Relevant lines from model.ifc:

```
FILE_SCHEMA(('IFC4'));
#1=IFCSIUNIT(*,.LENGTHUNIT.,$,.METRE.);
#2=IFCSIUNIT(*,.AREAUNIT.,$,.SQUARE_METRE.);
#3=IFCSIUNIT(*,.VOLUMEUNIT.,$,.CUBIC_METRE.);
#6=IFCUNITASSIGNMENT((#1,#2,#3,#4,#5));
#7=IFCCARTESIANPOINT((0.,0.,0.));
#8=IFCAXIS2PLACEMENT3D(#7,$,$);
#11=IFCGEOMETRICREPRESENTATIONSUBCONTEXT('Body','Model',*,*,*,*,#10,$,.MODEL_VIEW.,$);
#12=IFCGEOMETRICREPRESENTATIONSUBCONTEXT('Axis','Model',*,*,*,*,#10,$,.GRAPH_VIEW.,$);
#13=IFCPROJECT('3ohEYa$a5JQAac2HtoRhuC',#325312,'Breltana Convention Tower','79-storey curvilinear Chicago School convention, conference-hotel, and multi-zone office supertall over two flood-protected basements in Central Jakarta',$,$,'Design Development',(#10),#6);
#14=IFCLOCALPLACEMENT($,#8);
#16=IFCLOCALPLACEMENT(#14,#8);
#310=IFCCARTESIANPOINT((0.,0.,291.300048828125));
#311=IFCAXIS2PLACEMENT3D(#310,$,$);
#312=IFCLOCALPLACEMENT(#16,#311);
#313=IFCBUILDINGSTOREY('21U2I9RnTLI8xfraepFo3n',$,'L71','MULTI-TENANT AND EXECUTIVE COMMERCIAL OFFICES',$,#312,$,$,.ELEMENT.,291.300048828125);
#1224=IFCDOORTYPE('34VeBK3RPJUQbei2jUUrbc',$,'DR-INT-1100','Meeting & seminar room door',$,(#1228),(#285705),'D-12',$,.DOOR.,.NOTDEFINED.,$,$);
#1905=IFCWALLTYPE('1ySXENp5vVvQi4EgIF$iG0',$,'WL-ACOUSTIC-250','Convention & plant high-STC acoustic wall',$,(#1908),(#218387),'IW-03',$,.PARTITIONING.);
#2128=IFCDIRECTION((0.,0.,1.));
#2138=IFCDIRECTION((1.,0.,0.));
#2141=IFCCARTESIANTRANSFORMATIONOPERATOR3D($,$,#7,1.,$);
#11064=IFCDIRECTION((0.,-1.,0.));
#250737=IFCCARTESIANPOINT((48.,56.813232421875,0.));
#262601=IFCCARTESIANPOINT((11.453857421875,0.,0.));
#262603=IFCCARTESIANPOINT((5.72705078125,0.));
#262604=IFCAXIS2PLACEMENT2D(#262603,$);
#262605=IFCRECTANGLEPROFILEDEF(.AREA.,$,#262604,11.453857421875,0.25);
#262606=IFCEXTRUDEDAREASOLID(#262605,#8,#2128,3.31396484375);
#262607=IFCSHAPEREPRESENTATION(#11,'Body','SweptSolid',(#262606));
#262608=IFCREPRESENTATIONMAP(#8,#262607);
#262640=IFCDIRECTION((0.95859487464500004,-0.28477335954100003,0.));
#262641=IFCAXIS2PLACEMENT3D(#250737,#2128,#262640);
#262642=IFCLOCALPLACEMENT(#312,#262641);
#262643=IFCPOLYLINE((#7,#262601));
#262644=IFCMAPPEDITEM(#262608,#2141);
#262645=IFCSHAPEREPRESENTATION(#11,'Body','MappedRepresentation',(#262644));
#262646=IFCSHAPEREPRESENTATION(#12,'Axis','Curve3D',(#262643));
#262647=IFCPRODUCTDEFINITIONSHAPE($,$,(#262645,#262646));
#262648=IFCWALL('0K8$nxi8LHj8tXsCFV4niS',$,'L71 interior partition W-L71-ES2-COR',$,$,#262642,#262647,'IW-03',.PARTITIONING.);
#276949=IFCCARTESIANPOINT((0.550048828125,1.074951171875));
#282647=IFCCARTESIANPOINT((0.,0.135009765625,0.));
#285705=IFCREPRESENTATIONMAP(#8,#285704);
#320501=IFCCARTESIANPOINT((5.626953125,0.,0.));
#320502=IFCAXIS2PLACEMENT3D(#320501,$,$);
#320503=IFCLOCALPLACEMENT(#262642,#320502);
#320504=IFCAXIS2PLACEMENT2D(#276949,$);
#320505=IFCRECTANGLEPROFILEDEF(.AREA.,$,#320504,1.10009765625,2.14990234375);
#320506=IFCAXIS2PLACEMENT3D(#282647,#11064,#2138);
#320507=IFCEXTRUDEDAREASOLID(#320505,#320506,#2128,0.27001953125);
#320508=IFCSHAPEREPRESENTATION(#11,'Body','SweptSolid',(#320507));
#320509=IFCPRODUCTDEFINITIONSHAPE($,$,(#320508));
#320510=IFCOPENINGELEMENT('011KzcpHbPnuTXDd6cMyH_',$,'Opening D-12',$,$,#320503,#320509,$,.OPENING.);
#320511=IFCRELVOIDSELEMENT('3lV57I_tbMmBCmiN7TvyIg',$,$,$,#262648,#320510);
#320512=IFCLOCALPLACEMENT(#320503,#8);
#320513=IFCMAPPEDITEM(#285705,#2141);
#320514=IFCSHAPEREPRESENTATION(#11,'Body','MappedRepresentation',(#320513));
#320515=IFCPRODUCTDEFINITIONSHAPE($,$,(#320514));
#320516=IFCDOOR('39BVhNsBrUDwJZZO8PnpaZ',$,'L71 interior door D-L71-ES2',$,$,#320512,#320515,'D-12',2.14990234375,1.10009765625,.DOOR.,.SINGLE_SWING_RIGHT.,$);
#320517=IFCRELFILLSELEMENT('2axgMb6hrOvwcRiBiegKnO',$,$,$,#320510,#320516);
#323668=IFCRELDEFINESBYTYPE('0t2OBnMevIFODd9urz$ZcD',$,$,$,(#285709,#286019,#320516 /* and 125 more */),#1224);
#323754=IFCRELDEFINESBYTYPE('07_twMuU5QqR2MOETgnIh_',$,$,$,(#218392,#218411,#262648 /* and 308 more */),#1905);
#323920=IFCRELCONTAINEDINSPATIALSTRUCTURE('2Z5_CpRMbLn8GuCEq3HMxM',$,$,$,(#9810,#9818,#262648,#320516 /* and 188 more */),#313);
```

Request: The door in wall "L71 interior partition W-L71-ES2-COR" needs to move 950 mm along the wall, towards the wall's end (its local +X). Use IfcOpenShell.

```python
import ifcopenshell
import ifcopenshell.api.geometry
import ifcopenshell.util.placement
import ifcopenshell.util.unit

model = ifcopenshell.open("model.ifc")
unit_scale = ifcopenshell.util.unit.calculate_unit_scale(model)

door = model.by_id(320516)
opening = door.FillsVoids[0].RelatingOpeningElement
wall = opening.VoidsElements[0].RelatingBuildingElement

wall_matrix = ifcopenshell.util.placement.get_local_placement(wall.ObjectPlacement)
shift = wall_matrix[:3, 0] * 0.95 / unit_scale
before = ifcopenshell.util.placement.get_local_placement(door.ObjectPlacement)[:3, 3].copy()

# The door is placed relative to its opening, so it follows when the opening moves.
matrix = ifcopenshell.util.placement.get_local_placement(opening.ObjectPlacement)
matrix[:3, 3] += shift
ifcopenshell.api.geometry.edit_object_placement(
    model, product=opening, matrix=matrix, is_si=False, should_transform_children=True
)

after = ifcopenshell.util.placement.get_local_placement(door.ObjectPlacement)[:3, 3]
print("door moved by", (after - before).round(3) + 0.0)

model.write("model_rev.ifc")
```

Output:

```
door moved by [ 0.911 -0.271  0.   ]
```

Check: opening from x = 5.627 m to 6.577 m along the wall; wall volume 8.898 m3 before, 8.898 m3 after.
